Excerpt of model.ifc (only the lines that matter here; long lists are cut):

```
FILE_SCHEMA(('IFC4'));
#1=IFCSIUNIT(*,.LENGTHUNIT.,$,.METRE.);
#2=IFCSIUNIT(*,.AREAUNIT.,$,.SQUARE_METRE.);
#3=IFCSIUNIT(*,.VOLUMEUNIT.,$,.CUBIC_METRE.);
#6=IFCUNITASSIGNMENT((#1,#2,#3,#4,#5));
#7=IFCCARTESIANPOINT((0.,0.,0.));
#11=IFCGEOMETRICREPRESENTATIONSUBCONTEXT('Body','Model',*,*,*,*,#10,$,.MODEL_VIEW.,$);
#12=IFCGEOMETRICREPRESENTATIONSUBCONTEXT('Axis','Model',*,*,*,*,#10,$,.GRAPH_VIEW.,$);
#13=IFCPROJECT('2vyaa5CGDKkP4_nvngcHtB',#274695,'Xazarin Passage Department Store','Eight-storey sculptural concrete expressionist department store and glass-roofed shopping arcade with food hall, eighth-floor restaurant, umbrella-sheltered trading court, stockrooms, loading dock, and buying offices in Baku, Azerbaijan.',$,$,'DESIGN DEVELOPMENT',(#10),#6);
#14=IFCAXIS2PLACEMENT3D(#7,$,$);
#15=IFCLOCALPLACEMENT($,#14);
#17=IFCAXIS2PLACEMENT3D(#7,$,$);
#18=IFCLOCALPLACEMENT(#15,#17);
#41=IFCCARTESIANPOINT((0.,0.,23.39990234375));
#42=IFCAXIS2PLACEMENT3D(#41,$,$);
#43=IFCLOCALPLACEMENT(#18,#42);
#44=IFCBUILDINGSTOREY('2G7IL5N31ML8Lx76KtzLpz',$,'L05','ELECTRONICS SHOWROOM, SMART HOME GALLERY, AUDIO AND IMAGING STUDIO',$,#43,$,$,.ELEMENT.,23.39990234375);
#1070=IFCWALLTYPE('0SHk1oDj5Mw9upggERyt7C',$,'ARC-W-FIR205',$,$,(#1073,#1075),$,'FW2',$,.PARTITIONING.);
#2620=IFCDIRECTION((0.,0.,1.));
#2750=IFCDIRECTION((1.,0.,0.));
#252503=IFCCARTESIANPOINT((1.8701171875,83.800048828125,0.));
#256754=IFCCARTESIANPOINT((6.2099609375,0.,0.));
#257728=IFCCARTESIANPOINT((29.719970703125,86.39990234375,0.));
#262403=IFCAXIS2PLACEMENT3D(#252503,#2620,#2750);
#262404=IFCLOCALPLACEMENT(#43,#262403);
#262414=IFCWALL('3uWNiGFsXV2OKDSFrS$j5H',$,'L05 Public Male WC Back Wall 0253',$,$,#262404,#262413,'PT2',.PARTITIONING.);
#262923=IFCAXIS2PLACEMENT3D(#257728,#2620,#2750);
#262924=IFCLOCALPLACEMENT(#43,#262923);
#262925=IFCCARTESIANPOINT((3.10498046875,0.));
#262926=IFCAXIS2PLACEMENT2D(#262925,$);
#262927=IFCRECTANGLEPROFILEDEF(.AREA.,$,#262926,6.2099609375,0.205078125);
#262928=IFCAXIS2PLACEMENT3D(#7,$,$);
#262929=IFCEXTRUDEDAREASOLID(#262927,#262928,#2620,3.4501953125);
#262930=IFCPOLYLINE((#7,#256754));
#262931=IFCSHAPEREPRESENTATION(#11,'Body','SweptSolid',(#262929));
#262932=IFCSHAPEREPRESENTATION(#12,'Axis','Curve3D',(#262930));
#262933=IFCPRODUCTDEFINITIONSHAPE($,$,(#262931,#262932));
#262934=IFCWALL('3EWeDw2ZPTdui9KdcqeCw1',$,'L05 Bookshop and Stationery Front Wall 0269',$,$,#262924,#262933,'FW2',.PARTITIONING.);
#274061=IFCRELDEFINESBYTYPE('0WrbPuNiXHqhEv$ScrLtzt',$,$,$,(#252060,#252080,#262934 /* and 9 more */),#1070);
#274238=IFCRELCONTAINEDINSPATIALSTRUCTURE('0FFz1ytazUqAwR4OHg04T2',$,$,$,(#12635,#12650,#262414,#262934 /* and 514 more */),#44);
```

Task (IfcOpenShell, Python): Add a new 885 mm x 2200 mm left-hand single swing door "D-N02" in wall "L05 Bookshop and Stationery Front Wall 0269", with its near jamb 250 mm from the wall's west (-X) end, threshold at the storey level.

```python
import numpy as np
import ifcopenshell
import ifcopenshell.api.feature
import ifcopenshell.api.geometry
import ifcopenshell.api.root
import ifcopenshell.api.spatial
import ifcopenshell.geom
import ifcopenshell.util.element
import ifcopenshell.util.placement
import ifcopenshell.util.representation
import ifcopenshell.util.shape
import ifcopenshell.util.unit

model = ifcopenshell.open("model.ifc")
unit_scale = ifcopenshell.util.unit.calculate_unit_scale(model)
settings = ifcopenshell.geom.settings()


def volume(element):
    """Net volume in cubic metres, openings subtracted."""
    shape = ifcopenshell.geom.create_shape(settings, element)
    return ifcopenshell.util.shape.get_volume(shape.geometry)


wall = model.by_id(262934)
storey = ifcopenshell.util.element.get_container(wall, ifc_class="IfcBuildingStorey")
context = ifcopenshell.util.representation.get_context(model, "Model", "Body", "MODEL_VIEW")
before = volume(wall)

width, height, from_end, sill = 0.885, 2.2, 0.25, 0.0  # metres

# The wall runs along its own X axis, and the end named is its -X end.
wall_shape = ifcopenshell.geom.create_shape(settings, wall)
x, y, z = ifcopenshell.util.shape.get_vertices(wall_shape.geometry).T
start = x.min() + from_end
face, thickness = float(y.min()), float(y.max() - y.min())
wall_matrix = ifcopenshell.util.placement.get_local_placement(wall.ObjectPlacement)
level = ifcopenshell.util.placement.get_local_placement(storey.ObjectPlacement)[2, 3]


def in_wall(x, y):
    """Placement at x, y metres in the wall's axes, at sill height."""
    matrix = wall_matrix.copy()
    matrix[:, 3] = wall_matrix @ np.array([x / unit_scale, y / unit_scale, 0.0, 1.0])
    matrix[2, 3] = level + sill / unit_scale
    return matrix


# Opening: a box that overshoots both wall faces by 50 mm.
opening = ifcopenshell.api.root.create_entity(model, ifc_class="IfcOpeningElement", predefined_type="OPENING")
box = ifcopenshell.api.geometry.add_wall_representation(
    model, context=context, length=width, height=height, thickness=thickness + 0.1
)
ifcopenshell.api.geometry.assign_representation(model, product=opening, representation=box)
ifcopenshell.api.geometry.edit_object_placement(model, product=opening, matrix=in_wall(start, face - 0.05), is_si=False)
ifcopenshell.api.feature.add_feature(model, feature=opening, element=wall)

door = ifcopenshell.api.root.create_entity(model, ifc_class="IfcDoor", name="D-N02", predefined_type="DOOR")
door.OverallWidth, door.OverallHeight = width / unit_scale, height / unit_scale
door.OperationType = "SINGLE_SWING_LEFT"
body = ifcopenshell.api.geometry.add_door_representation(
    model,
    context=context,
    overall_width=door.OverallWidth,
    overall_height=door.OverallHeight,
    operation_type="SINGLE_SWING_LEFT",
    lining_properties={"LiningDepth": thickness / unit_scale, "ThresholdDepth": thickness / unit_scale},
)
ifcopenshell.api.geometry.assign_representation(model, product=door, representation=body)
ifcopenshell.api.spatial.assign_container(model, products=[door], relating_structure=storey)
ifcopenshell.api.feature.add_filling(model, opening=opening, element=door)

# The lining spans the wall, so the door starts at the wall face.
ifcopenshell.api.geometry.edit_object_placement(model, product=door, matrix=in_wall(start, face), is_si=False)

after = volume(wall)

print(f"wall volume {before:.3f} -> {after:.3f} m3")

model.write("model_rev.ifc")
```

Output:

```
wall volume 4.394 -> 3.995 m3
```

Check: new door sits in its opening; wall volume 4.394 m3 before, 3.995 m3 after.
